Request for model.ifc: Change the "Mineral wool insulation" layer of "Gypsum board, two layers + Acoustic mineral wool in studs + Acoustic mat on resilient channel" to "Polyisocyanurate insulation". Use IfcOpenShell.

First a look at what the model holds.

```python
import ifcopenshell
import ifcopenshell.util.element

model = ifcopenshell.open("model.ifc")
print(model.schema)
for layer_set in model.by_type("IfcMaterialLayerSet"):
    if layer_set.LayerSetName == "Gypsum board, two layers + Acoustic mineral wool in studs + Acoustic mat on resilient channel":
        for layer in layer_set.MaterialLayers:
            print(layer.id(), layer.Material and layer.Material.Name, layer.LayerThickness, sep=" | ")
        print(len(ifcopenshell.util.element.get_elements_by_material(model, layer_set)), "elements and types use it")
print(sorted(m.Name for m in model.by_type("IfcMaterial") if m.Name)[:60])
```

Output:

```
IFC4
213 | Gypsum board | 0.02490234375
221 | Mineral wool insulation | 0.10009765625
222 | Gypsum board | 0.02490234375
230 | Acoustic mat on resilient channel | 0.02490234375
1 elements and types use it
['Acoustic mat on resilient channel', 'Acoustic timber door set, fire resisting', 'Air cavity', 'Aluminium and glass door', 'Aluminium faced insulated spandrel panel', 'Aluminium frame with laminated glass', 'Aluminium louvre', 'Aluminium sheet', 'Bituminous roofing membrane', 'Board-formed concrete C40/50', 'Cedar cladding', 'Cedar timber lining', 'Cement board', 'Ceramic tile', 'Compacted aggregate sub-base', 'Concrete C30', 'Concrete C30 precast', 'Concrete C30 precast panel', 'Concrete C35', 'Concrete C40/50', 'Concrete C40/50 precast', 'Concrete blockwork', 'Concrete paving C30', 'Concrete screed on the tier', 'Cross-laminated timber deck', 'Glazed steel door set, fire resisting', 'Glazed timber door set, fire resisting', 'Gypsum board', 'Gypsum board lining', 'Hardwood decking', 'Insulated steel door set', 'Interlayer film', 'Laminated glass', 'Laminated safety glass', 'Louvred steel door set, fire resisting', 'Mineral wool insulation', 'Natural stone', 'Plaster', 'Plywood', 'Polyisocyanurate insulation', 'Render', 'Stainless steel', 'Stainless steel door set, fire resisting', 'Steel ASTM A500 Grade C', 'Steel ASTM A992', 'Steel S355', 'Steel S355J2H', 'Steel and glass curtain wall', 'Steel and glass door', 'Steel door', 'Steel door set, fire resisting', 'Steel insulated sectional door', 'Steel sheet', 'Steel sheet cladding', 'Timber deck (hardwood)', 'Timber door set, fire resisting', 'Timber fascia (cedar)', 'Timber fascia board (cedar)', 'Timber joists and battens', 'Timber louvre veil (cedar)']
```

```python
import ifcopenshell
import ifcopenshell.api.material

model = ifcopenshell.open("model.ifc")

layer_set = next(s for s in model.by_type("IfcMaterialLayerSet") if s.LayerSetName == "Gypsum board, two layers + Acoustic mineral wool in studs + Acoustic mat on resilient channel")
layer = next(l for l in layer_set.MaterialLayers if l.Material and l.Material.Name == "Mineral wool insulation")
material = next(m for m in model.by_type("IfcMaterial") if m.Name == "Polyisocyanurate insulation")

# Point this one layer at the other material; renaming the old one would change it everywhere.
ifcopenshell.api.material.edit_layer(model, layer=layer, attributes={}, material=material)

print([l.Material.Name if l.Material else None for l in layer_set.MaterialLayers])

model.write("model-out.ifc")
```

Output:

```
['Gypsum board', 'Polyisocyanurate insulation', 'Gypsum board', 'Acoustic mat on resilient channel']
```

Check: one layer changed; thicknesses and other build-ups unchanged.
